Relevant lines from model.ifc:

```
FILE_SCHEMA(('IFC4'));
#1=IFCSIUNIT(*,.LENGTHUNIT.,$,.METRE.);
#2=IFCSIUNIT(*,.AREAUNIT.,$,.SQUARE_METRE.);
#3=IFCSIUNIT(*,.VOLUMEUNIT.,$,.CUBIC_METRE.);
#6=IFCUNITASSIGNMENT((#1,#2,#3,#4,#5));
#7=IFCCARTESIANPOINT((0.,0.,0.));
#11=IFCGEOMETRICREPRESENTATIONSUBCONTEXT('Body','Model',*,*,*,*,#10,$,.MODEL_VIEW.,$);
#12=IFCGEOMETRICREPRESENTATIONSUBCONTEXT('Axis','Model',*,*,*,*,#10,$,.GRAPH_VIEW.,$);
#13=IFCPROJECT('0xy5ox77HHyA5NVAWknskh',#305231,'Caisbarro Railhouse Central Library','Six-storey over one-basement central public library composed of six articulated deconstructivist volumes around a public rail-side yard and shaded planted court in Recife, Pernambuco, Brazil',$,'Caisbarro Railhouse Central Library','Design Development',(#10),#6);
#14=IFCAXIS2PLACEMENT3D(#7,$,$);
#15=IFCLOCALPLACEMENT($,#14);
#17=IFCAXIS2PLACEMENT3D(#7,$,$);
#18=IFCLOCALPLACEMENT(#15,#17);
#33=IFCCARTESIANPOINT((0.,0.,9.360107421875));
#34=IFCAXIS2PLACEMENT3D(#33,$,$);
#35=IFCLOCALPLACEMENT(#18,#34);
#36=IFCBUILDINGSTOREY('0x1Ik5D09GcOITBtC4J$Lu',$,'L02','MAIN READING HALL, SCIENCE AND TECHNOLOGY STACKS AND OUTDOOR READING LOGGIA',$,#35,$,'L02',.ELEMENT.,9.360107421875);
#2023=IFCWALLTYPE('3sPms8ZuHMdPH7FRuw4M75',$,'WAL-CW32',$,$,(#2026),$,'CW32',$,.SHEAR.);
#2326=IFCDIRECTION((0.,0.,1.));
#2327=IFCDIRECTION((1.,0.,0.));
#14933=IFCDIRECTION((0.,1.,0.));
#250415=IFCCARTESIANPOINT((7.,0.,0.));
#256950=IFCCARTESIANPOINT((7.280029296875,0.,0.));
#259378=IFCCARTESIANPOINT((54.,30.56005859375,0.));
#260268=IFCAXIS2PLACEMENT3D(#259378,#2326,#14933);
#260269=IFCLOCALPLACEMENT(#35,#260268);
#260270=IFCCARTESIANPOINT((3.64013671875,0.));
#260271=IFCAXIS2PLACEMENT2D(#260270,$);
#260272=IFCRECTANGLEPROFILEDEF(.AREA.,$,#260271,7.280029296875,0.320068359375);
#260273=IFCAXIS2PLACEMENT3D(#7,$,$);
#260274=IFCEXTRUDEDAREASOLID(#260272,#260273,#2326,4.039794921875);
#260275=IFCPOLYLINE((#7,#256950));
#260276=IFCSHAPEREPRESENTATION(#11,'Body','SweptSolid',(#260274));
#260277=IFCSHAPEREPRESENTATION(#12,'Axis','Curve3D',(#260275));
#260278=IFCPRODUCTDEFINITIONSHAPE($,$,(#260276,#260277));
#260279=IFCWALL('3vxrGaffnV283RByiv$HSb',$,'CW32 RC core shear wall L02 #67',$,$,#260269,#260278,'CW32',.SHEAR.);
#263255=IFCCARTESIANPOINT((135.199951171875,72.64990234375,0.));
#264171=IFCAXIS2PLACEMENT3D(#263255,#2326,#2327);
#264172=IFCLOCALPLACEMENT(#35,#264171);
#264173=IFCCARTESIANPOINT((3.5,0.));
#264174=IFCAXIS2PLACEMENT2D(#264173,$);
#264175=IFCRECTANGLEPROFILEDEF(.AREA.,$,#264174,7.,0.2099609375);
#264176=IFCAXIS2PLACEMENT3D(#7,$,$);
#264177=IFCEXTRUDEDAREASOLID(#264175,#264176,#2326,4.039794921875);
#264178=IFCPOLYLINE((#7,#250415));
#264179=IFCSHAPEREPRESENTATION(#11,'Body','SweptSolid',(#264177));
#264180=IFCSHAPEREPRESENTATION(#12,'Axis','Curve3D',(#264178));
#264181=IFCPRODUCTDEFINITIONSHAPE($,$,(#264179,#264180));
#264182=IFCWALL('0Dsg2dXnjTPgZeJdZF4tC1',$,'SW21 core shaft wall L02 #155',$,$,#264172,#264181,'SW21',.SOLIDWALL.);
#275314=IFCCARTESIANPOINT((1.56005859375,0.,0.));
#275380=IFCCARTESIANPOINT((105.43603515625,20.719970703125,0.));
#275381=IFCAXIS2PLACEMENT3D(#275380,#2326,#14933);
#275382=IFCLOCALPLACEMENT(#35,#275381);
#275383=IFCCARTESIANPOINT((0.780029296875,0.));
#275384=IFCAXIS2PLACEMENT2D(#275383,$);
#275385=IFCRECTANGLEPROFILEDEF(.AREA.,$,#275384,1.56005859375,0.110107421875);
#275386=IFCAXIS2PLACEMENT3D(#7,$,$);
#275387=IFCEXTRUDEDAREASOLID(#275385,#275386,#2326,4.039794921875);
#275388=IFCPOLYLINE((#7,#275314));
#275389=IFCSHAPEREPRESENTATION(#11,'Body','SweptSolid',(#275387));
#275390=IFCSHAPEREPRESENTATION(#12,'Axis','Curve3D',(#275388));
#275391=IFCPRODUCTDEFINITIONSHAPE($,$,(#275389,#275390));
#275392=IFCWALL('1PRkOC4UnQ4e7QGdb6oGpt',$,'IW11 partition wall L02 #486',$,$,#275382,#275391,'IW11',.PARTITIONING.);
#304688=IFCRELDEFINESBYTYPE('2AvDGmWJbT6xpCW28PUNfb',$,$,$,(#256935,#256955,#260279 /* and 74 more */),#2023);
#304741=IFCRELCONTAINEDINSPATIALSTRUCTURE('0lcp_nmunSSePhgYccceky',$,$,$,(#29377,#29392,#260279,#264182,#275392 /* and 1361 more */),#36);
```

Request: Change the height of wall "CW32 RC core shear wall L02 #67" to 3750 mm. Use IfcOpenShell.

```python
import ifcopenshell
import ifcopenshell.geom
import ifcopenshell.util.representation
import ifcopenshell.util.shape
import ifcopenshell.util.unit

model = ifcopenshell.open("model.ifc")
unit_scale = ifcopenshell.util.unit.calculate_unit_scale(model)
settings = ifcopenshell.geom.settings()


def volume(element):
    """Net volume in cubic metres, openings subtracted."""
    shape = ifcopenshell.geom.create_shape(settings, element)
    return ifcopenshell.util.shape.get_volume(shape.geometry)


wall = model.by_guid("3vxrGaffnV283RByiv$HSb")
before = volume(wall)

body = ifcopenshell.util.representation.get_representation(wall, "Model", "Body")
solid = body.Items[0]
old_height = solid.Depth
solid.Depth = 3.75 / unit_scale
after = volume(wall)

print(f"height {old_height:g} -> {solid.Depth:g}, volume {before:.3f} -> {after:.3f} m3")

model.write("model-out.ifc")
```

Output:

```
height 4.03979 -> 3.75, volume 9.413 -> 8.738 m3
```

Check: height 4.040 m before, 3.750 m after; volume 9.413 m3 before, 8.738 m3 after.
